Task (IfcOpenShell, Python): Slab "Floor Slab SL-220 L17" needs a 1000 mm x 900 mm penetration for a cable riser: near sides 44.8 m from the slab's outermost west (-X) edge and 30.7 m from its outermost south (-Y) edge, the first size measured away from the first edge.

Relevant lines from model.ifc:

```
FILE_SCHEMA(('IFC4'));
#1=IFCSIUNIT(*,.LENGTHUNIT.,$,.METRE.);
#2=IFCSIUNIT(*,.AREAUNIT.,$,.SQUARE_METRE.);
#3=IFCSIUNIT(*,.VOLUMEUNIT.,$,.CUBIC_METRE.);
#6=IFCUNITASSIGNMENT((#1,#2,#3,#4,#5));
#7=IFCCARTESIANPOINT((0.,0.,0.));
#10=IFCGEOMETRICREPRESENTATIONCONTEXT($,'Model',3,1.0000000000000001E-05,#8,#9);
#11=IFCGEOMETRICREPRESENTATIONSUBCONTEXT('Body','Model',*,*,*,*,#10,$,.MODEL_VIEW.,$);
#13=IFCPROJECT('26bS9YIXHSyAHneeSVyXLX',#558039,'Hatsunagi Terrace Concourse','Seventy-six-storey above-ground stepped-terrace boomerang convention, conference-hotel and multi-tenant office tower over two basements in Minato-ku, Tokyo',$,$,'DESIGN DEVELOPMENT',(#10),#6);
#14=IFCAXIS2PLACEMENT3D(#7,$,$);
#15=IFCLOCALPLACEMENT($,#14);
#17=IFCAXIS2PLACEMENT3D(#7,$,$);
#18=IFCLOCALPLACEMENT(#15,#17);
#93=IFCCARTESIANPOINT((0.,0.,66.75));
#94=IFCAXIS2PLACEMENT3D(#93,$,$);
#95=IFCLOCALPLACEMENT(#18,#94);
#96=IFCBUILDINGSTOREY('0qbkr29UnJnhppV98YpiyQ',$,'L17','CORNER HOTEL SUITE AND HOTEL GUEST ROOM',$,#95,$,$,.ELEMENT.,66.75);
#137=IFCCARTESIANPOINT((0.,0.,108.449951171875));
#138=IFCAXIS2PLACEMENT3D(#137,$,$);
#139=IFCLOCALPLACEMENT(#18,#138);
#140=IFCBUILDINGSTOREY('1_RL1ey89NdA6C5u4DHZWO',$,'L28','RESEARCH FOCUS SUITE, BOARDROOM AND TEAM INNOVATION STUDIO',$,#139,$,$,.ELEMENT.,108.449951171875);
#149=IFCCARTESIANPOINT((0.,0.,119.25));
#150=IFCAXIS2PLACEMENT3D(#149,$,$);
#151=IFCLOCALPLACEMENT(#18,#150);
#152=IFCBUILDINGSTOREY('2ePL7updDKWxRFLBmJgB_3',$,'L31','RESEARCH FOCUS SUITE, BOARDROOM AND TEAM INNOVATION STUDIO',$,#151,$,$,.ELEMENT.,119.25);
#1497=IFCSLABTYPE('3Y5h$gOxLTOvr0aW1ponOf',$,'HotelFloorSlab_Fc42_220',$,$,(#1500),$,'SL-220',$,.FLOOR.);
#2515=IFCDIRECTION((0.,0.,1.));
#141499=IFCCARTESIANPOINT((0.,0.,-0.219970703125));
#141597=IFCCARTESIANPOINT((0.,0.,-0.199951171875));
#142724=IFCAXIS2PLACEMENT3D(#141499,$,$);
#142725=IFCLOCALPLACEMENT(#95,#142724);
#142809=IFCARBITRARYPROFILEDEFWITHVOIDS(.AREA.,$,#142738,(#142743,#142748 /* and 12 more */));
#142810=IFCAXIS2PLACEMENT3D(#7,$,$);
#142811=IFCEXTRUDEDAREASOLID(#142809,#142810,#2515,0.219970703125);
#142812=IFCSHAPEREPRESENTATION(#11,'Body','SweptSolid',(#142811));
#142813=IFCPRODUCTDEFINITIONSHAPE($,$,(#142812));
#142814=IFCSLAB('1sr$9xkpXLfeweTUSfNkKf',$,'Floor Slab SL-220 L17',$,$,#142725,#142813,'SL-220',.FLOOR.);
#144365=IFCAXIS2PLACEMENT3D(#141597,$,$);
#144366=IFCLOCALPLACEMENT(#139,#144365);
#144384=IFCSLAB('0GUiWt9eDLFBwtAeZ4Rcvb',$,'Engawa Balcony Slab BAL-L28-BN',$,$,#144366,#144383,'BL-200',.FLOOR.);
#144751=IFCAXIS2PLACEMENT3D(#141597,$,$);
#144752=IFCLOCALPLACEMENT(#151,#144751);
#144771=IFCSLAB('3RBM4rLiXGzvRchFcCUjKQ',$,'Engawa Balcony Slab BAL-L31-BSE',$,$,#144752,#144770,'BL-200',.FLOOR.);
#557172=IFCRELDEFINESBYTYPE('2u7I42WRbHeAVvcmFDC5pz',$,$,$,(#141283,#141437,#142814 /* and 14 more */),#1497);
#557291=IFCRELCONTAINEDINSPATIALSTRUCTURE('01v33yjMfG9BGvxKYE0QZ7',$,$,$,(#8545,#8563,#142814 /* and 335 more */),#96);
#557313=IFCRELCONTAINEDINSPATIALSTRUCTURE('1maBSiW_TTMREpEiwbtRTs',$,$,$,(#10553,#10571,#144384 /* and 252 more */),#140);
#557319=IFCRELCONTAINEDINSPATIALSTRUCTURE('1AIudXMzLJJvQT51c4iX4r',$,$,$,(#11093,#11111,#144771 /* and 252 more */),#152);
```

```python
import numpy as np
import ifcopenshell
import ifcopenshell.api.feature
import ifcopenshell.api.geometry
import ifcopenshell.api.root
import ifcopenshell.geom
import ifcopenshell.util.placement
import ifcopenshell.util.representation
import ifcopenshell.util.shape
import ifcopenshell.util.unit

model = ifcopenshell.open("model.ifc")
unit_scale = ifcopenshell.util.unit.calculate_unit_scale(model)
settings = ifcopenshell.geom.settings()


def volume(element):
    """Net volume in cubic metres, openings subtracted."""
    shape = ifcopenshell.geom.create_shape(settings, element)
    return ifcopenshell.util.shape.get_volume(shape.geometry)


slab = model.by_guid("1sr$9xkpXLfeweTUSfNkKf")
before = volume(slab)

# Extent in the slab's own axes, in metres. The edges named are its -X and -Y sides.
slab_shape = ifcopenshell.geom.create_shape(settings, slab)
vertices = ifcopenshell.util.shape.get_vertices(slab_shape.geometry)
x_min, y_min, bottom = vertices.min(axis=0)
top = vertices[:, 2].max()

opening = ifcopenshell.api.root.create_entity(model, ifc_class="IfcOpeningElement", name="Cable riser opening", predefined_type="OPENING")
context = ifcopenshell.util.representation.get_context(model, "Model", "Body", "MODEL_VIEW")
width, depth = 1, 0.9
outline = [(0.0, 0.0), (width, 0.0), (width, depth), (0.0, depth), (0.0, 0.0)]
# Overshoot both faces by 50 mm so the cut is clean.
shape = ifcopenshell.api.geometry.add_slab_representation(
    model, context=context, depth=top - bottom + 0.1, polyline=outline
)
ifcopenshell.api.geometry.assign_representation(model, product=opening, representation=shape)

matrix = ifcopenshell.util.placement.get_local_placement(slab.ObjectPlacement)
matrix[:, 3] = matrix @ np.append(np.array([x_min + 44.8, y_min + 30.7, bottom - 0.05]) / unit_scale, 1.0)
ifcopenshell.api.geometry.edit_object_placement(model, product=opening, matrix=matrix, is_si=False)
ifcopenshell.api.feature.add_feature(model, feature=opening, element=slab)

after = volume(slab)

print(f"slab volume {before:.3f} -> {after:.3f} m3")

model.write("model_rev.ifc")
```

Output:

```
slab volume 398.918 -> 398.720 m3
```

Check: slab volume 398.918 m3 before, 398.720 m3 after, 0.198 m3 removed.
